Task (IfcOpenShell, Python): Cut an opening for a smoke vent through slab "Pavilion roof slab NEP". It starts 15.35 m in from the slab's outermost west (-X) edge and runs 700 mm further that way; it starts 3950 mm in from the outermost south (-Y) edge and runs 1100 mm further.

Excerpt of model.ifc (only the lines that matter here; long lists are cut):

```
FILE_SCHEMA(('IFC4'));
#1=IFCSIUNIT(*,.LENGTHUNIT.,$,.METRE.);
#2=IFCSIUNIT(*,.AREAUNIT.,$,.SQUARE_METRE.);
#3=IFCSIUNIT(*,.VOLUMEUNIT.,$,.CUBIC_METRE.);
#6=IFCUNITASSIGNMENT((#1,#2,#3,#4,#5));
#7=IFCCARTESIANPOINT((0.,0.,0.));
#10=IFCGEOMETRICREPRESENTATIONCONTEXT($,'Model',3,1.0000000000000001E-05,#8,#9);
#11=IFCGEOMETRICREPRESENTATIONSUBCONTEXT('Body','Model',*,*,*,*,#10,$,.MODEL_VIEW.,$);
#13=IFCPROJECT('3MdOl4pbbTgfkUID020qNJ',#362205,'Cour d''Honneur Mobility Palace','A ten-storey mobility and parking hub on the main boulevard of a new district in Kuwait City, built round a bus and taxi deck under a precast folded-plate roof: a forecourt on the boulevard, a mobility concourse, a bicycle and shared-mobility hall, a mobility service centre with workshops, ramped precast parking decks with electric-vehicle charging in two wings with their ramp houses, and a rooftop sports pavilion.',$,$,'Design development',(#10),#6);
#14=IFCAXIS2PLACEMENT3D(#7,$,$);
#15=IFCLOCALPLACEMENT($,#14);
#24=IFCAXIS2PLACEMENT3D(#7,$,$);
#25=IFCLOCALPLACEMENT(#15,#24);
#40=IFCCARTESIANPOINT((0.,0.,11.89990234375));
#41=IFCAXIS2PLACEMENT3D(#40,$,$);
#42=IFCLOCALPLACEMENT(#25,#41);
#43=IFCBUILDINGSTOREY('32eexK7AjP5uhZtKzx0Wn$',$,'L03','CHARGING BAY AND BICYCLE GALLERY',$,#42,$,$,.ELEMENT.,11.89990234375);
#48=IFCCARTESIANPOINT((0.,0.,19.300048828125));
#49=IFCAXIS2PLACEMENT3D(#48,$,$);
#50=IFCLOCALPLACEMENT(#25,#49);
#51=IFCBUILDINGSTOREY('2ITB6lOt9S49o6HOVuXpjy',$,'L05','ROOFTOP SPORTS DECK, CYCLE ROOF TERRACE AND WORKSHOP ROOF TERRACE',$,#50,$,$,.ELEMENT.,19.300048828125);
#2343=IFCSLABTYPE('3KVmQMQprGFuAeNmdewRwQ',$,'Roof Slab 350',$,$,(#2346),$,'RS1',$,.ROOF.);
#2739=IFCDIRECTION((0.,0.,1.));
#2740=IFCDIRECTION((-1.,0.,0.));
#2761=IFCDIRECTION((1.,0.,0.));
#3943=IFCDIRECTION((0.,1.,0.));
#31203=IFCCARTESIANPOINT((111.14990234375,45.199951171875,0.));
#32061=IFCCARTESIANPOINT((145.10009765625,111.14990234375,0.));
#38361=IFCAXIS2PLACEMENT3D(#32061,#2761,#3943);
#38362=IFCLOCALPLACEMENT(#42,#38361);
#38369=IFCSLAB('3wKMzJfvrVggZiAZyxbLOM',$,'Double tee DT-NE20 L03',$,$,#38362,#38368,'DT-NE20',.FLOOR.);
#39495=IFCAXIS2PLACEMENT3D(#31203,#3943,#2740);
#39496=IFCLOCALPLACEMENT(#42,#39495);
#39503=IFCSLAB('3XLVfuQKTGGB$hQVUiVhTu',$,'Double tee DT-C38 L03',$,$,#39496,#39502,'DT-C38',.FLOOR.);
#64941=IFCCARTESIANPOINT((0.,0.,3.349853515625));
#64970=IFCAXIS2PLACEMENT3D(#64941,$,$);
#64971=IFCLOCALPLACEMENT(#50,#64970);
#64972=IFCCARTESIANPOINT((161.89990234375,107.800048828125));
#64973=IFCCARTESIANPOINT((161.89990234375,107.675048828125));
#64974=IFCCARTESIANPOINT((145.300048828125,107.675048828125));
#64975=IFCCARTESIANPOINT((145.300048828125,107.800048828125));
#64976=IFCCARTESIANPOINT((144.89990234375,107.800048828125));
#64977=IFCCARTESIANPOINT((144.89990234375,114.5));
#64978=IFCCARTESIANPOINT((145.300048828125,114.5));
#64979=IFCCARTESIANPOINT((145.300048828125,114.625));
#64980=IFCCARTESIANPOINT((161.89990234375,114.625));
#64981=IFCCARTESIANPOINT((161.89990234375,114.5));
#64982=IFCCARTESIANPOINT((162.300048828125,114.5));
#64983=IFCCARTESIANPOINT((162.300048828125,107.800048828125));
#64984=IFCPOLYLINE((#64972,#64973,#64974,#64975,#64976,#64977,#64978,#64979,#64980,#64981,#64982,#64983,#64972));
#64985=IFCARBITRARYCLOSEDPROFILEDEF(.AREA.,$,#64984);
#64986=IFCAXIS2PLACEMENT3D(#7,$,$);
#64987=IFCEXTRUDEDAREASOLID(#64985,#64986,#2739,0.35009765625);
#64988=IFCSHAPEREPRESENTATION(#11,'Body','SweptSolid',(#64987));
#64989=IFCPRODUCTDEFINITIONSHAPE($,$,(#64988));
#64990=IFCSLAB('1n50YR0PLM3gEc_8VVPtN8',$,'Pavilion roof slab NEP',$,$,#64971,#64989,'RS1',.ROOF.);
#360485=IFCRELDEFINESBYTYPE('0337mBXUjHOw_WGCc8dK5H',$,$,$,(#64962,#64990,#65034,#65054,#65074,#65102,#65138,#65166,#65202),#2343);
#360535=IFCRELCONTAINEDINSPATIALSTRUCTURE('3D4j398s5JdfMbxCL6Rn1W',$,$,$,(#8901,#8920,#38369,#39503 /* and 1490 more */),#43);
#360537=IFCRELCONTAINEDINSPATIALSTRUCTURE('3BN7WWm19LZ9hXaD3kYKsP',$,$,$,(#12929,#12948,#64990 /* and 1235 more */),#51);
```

```python
import numpy as np
import ifcopenshell
import ifcopenshell.api.feature
import ifcopenshell.api.geometry
import ifcopenshell.api.root
import ifcopenshell.geom
import ifcopenshell.util.placement
import ifcopenshell.util.representation
import ifcopenshell.util.shape
import ifcopenshell.util.unit

model = ifcopenshell.open("model.ifc")
unit_scale = ifcopenshell.util.unit.calculate_unit_scale(model)
settings = ifcopenshell.geom.settings()


def volume(element):
    """Net volume in cubic metres, openings subtracted."""
    shape = ifcopenshell.geom.create_shape(settings, element)
    return ifcopenshell.util.shape.get_volume(shape.geometry)


slab = model.by_guid("1n50YR0PLM3gEc_8VVPtN8")
before = volume(slab)

# Extent in the slab's own axes, in metres. The edges named are its -X and -Y sides.
slab_shape = ifcopenshell.geom.create_shape(settings, slab)
vertices = ifcopenshell.util.shape.get_vertices(slab_shape.geometry)
x_min, y_min, bottom = vertices.min(axis=0)
top = vertices[:, 2].max()

opening = ifcopenshell.api.root.create_entity(model, ifc_class="IfcOpeningElement", name="Smoke vent opening", predefined_type="OPENING")
context = ifcopenshell.util.representation.get_context(model, "Model", "Body", "MODEL_VIEW")
width, depth = 0.7, 1.1
outline = [(0.0, 0.0), (width, 0.0), (width, depth), (0.0, depth), (0.0, 0.0)]
# Overshoot both faces by 50 mm so the cut is clean.
shape = ifcopenshell.api.geometry.add_slab_representation(
    model, context=context, depth=top - bottom + 0.1, polyline=outline
)
ifcopenshell.api.geometry.assign_representation(model, product=opening, representation=shape)

matrix = ifcopenshell.util.placement.get_local_placement(slab.ObjectPlacement)
matrix[:, 3] = matrix @ np.append(np.array([x_min + 15.35, y_min + 3.95, bottom - 0.05]) / unit_scale, 1.0)
ifcopenshell.api.geometry.edit_object_placement(model, product=opening, matrix=matrix, is_si=False)
ifcopenshell.api.feature.add_feature(model, feature=opening, element=slab)

after = volume(slab)

print(f"slab volume {before:.3f} -> {after:.3f} m3")

model.write("model_edited.ifc")
```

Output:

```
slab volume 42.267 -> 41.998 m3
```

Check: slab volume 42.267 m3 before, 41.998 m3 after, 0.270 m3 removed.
